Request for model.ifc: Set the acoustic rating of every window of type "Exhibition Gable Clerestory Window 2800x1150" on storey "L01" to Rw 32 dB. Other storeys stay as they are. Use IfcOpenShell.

First a look at what the model holds.

```python
import ifcopenshell
import ifcopenshell.util.element

model = ifcopenshell.open("model.ifc")
print(model.schema)
storey = next(s for s in model.by_type("IfcBuildingStorey") if s.Name == "L01")
windows = [e for e in ifcopenshell.util.element.get_decomposition(storey) if e.is_a("IfcWindow")]
seen = {}
for e in windows:
    element_type = ifcopenshell.util.element.get_type(e)
    key = (element_type.Name if element_type != e and element_type else None, ifcopenshell.util.element.get_pset(e, "Pset_WindowCommon", "AcousticRating"))
    seen[key] = seen.get(key, 0) + 1
for (name, value), count in sorted(seen.items(), key=str):
    print(count, "x", name, "|", value)
```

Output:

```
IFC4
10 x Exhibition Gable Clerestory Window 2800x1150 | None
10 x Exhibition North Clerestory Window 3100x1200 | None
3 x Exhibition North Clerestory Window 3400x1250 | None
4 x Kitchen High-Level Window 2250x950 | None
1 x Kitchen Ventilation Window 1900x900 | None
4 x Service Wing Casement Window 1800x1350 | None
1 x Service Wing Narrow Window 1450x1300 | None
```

```python
import ifcopenshell
import ifcopenshell.api.pset
import ifcopenshell.util.element

model = ifcopenshell.open("model.ifc")

storey = next(s for s in model.by_type("IfcBuildingStorey") if s.Name == "L01")
windows = [e for e in ifcopenshell.util.element.get_decomposition(storey) if e.is_a("IfcWindow")]

count = 0
for e in windows:
    element_type = ifcopenshell.util.element.get_type(e)
    if element_type in (None, e) or element_type.Name != "Exhibition Gable Clerestory Window 2800x1150":
        continue
    # add_pset returns the element's existing set when there is one.
    pset = ifcopenshell.api.pset.add_pset(model, product=e, name="Pset_WindowCommon")
    ifcopenshell.api.pset.edit_pset(model, pset=pset, properties={"AcousticRating": "Rw 32 dB"})
    count += 1

print(count, "windows updated")

model.write("model_updated.ifc")
```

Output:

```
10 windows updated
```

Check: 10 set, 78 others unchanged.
